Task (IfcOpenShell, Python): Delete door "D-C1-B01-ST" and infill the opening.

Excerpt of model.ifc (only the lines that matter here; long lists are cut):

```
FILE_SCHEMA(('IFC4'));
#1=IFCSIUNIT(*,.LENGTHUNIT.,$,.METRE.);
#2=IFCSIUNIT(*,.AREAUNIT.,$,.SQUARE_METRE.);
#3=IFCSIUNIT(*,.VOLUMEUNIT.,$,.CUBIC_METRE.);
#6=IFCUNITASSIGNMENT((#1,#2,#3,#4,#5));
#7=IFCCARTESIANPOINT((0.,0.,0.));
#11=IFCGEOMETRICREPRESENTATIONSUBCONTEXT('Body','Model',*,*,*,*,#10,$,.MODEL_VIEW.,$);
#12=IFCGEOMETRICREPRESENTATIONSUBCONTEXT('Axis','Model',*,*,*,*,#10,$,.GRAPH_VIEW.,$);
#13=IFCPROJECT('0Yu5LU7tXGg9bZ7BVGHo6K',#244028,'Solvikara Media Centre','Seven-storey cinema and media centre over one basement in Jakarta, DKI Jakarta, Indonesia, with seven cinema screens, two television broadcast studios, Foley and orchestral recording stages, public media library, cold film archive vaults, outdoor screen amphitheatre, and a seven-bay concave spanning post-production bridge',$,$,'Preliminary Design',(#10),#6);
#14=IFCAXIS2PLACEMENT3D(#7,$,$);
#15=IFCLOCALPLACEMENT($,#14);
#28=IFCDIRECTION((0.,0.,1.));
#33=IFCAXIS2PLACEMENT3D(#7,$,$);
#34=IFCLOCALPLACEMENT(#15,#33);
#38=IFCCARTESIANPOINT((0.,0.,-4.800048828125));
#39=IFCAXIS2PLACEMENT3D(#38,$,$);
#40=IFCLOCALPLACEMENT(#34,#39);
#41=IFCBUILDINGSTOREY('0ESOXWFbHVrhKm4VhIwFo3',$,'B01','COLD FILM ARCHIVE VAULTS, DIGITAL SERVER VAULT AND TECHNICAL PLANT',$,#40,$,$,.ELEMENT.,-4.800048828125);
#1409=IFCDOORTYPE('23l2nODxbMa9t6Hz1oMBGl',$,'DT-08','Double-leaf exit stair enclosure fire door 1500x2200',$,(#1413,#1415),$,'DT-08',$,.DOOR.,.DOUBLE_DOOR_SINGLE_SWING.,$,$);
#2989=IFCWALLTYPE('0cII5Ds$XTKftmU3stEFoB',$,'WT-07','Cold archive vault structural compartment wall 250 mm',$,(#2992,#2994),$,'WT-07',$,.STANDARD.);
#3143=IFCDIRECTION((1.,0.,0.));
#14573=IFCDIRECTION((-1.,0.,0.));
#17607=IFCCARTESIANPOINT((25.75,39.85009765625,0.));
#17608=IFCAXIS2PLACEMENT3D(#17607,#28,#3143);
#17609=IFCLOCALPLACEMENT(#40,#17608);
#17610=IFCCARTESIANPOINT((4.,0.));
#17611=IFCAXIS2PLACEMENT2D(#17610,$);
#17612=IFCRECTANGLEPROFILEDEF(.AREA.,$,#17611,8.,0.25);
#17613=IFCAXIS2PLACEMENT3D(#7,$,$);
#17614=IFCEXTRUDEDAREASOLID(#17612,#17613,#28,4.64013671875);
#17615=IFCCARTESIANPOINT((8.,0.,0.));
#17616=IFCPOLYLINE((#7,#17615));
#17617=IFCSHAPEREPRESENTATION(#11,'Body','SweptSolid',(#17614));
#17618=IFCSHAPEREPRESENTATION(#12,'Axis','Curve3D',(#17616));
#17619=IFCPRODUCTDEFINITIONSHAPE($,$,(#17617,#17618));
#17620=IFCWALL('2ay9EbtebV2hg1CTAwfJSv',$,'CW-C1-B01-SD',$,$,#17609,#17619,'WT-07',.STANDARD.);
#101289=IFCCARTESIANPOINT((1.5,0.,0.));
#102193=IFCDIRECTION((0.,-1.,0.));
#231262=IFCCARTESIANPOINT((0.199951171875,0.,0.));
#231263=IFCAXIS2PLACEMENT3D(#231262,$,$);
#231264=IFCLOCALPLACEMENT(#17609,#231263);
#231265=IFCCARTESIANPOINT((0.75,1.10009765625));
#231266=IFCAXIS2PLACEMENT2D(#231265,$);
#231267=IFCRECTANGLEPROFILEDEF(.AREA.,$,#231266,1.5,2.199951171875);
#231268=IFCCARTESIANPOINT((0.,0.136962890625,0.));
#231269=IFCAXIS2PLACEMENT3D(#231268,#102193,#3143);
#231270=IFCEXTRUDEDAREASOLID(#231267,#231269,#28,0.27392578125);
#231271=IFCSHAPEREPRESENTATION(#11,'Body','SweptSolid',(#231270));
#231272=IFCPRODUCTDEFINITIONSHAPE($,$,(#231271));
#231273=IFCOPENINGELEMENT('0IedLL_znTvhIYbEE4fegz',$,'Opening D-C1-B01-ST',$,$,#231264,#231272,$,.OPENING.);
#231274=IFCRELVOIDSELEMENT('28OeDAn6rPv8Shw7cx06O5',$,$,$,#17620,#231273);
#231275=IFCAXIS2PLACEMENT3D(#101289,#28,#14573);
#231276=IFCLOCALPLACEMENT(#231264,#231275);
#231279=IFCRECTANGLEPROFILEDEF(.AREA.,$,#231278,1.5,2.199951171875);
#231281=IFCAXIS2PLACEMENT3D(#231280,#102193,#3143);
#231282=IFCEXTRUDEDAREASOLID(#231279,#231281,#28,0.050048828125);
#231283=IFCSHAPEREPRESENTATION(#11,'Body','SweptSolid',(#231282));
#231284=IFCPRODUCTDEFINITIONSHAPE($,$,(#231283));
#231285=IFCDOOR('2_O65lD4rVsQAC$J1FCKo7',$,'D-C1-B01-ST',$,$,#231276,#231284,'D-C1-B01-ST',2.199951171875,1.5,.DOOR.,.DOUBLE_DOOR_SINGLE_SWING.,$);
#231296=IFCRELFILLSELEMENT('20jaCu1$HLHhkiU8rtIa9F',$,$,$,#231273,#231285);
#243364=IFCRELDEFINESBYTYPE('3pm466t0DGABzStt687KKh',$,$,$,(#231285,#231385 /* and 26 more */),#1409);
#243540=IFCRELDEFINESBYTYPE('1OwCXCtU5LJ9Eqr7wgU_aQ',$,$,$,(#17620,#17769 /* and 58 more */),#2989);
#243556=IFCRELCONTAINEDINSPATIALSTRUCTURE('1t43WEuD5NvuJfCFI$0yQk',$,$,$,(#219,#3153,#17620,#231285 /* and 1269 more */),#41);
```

```python
import ifcopenshell
import ifcopenshell.api.feature
import ifcopenshell.api.root
import ifcopenshell.geom
import ifcopenshell.util.shape

model = ifcopenshell.open("model.ifc")
settings = ifcopenshell.geom.settings()


def volume(element):
    """Net volume in cubic metres, openings subtracted."""
    shape = ifcopenshell.geom.create_shape(settings, element)
    return ifcopenshell.util.shape.get_volume(shape.geometry)


door = model.by_guid("2_O65lD4rVsQAC$J1FCKo7")
opening = door.FillsVoids[0].RelatingOpeningElement
wall = opening.VoidsElements[0].RelatingBuildingElement
before = volume(wall)

ifcopenshell.api.root.remove_product(model, product=door)
ifcopenshell.api.feature.remove_feature(model, feature=opening)

after = volume(wall)

print(f"wall volume {before:.3f} -> {after:.3f} m3")

model.write("model_v2.ifc")
```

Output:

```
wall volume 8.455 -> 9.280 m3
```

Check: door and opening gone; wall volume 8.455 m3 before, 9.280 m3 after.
